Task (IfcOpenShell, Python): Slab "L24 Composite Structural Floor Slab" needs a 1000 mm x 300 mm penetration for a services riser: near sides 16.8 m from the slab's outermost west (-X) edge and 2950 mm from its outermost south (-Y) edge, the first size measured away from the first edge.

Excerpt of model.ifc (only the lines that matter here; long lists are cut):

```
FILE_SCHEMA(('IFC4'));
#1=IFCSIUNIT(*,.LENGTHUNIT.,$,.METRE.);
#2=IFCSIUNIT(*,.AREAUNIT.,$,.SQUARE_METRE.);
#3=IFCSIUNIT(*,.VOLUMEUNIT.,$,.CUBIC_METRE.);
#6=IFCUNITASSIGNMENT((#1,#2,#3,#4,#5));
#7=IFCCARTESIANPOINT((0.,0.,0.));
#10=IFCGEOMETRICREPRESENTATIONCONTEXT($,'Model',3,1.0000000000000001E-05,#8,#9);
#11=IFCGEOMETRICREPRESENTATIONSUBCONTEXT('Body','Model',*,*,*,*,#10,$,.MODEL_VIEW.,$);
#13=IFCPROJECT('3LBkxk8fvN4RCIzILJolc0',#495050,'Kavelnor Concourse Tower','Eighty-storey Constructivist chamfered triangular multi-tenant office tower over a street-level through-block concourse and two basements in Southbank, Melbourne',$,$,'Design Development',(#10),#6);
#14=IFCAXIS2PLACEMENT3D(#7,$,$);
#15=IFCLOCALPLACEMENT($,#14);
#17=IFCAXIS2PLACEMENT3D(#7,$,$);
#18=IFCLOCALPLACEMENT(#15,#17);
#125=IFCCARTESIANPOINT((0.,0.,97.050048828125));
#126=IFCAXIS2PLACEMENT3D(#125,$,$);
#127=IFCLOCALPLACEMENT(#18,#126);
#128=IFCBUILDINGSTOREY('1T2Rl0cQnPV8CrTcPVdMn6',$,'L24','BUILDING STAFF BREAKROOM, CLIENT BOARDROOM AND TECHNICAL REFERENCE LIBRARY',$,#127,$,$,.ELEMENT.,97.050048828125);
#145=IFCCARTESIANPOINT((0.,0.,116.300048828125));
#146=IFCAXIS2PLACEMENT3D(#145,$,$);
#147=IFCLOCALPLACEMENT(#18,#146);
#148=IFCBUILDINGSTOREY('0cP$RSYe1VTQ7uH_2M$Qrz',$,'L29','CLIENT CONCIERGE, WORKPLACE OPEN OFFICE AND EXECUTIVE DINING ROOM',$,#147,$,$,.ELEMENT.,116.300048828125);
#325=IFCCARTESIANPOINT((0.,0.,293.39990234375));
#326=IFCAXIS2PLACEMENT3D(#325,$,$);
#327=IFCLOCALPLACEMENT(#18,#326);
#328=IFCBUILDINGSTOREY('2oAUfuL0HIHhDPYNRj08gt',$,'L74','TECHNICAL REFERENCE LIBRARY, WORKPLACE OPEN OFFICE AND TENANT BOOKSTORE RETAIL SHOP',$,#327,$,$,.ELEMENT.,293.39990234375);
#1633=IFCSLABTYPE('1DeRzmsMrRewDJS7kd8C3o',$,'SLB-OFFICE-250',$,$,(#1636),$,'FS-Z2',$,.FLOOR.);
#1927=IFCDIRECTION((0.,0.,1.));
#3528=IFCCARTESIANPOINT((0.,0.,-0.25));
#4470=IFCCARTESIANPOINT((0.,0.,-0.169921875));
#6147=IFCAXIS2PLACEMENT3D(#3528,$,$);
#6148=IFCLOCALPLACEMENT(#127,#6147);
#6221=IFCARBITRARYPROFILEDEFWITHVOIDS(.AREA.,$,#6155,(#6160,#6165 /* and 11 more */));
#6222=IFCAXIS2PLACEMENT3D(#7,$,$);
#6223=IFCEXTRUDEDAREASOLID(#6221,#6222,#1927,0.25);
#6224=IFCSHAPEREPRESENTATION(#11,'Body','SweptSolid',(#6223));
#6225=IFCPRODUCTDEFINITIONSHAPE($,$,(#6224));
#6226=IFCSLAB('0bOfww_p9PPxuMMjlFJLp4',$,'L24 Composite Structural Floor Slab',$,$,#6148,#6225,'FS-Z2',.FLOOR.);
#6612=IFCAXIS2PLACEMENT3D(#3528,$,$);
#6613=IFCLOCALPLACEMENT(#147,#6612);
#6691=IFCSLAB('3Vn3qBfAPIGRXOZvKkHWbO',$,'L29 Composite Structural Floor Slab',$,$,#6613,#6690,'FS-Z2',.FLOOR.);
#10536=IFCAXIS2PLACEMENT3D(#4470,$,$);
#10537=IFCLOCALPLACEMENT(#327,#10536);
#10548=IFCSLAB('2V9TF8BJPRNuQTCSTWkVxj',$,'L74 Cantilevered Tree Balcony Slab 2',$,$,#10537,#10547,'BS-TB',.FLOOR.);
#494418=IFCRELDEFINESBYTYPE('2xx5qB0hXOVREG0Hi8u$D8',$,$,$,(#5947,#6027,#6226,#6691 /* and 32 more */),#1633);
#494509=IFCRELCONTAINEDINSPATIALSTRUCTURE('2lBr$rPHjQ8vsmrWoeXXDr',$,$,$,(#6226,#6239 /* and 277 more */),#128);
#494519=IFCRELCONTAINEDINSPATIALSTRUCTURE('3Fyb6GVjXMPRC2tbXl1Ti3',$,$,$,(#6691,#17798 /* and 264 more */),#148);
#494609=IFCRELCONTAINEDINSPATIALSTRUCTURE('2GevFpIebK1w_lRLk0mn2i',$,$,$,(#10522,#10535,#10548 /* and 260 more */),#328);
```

```python
import numpy as np
import ifcopenshell
import ifcopenshell.api.feature
import ifcopenshell.api.geometry
import ifcopenshell.api.root
import ifcopenshell.geom
import ifcopenshell.util.placement
import ifcopenshell.util.representation
import ifcopenshell.util.shape
import ifcopenshell.util.unit

model = ifcopenshell.open("model.ifc")
unit_scale = ifcopenshell.util.unit.calculate_unit_scale(model)
settings = ifcopenshell.geom.settings()


def volume(element):
    """Net volume in cubic metres, openings subtracted."""
    shape = ifcopenshell.geom.create_shape(settings, element)
    return ifcopenshell.util.shape.get_volume(shape.geometry)


slab = model.by_id(6226)
before = volume(slab)

# Extent in the slab's own axes, in metres. The edges named are its -X and -Y sides.
slab_shape = ifcopenshell.geom.create_shape(settings, slab)
vertices = ifcopenshell.util.shape.get_vertices(slab_shape.geometry)
x_min, y_min, bottom = vertices.min(axis=0)
top = vertices[:, 2].max()

opening = ifcopenshell.api.root.create_entity(model, ifc_class="IfcOpeningElement", name="Services riser opening", predefined_type="OPENING")
context = ifcopenshell.util.representation.get_context(model, "Model", "Body", "MODEL_VIEW")
width, depth = 1, 0.3
outline = [(0.0, 0.0), (width, 0.0), (width, depth), (0.0, depth), (0.0, 0.0)]
# Overshoot both faces by 50 mm so the cut is clean.
shape = ifcopenshell.api.geometry.add_slab_representation(
    model, context=context, depth=top - bottom + 0.1, polyline=outline
)
ifcopenshell.api.geometry.assign_representation(model, product=opening, representation=shape)

matrix = ifcopenshell.util.placement.get_local_placement(slab.ObjectPlacement)
matrix[:, 3] = matrix @ np.append(np.array([x_min + 16.8, y_min + 2.95, bottom - 0.05]) / unit_scale, 1.0)
ifcopenshell.api.geometry.edit_object_placement(model, product=opening, matrix=matrix, is_si=False)
ifcopenshell.api.feature.add_feature(model, feature=opening, element=slab)

after = volume(slab)

print(f"slab volume {before:.3f} -> {after:.3f} m3")

model.write("model_updated.ifc")
```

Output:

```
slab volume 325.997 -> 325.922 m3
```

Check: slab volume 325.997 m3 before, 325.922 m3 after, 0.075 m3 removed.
